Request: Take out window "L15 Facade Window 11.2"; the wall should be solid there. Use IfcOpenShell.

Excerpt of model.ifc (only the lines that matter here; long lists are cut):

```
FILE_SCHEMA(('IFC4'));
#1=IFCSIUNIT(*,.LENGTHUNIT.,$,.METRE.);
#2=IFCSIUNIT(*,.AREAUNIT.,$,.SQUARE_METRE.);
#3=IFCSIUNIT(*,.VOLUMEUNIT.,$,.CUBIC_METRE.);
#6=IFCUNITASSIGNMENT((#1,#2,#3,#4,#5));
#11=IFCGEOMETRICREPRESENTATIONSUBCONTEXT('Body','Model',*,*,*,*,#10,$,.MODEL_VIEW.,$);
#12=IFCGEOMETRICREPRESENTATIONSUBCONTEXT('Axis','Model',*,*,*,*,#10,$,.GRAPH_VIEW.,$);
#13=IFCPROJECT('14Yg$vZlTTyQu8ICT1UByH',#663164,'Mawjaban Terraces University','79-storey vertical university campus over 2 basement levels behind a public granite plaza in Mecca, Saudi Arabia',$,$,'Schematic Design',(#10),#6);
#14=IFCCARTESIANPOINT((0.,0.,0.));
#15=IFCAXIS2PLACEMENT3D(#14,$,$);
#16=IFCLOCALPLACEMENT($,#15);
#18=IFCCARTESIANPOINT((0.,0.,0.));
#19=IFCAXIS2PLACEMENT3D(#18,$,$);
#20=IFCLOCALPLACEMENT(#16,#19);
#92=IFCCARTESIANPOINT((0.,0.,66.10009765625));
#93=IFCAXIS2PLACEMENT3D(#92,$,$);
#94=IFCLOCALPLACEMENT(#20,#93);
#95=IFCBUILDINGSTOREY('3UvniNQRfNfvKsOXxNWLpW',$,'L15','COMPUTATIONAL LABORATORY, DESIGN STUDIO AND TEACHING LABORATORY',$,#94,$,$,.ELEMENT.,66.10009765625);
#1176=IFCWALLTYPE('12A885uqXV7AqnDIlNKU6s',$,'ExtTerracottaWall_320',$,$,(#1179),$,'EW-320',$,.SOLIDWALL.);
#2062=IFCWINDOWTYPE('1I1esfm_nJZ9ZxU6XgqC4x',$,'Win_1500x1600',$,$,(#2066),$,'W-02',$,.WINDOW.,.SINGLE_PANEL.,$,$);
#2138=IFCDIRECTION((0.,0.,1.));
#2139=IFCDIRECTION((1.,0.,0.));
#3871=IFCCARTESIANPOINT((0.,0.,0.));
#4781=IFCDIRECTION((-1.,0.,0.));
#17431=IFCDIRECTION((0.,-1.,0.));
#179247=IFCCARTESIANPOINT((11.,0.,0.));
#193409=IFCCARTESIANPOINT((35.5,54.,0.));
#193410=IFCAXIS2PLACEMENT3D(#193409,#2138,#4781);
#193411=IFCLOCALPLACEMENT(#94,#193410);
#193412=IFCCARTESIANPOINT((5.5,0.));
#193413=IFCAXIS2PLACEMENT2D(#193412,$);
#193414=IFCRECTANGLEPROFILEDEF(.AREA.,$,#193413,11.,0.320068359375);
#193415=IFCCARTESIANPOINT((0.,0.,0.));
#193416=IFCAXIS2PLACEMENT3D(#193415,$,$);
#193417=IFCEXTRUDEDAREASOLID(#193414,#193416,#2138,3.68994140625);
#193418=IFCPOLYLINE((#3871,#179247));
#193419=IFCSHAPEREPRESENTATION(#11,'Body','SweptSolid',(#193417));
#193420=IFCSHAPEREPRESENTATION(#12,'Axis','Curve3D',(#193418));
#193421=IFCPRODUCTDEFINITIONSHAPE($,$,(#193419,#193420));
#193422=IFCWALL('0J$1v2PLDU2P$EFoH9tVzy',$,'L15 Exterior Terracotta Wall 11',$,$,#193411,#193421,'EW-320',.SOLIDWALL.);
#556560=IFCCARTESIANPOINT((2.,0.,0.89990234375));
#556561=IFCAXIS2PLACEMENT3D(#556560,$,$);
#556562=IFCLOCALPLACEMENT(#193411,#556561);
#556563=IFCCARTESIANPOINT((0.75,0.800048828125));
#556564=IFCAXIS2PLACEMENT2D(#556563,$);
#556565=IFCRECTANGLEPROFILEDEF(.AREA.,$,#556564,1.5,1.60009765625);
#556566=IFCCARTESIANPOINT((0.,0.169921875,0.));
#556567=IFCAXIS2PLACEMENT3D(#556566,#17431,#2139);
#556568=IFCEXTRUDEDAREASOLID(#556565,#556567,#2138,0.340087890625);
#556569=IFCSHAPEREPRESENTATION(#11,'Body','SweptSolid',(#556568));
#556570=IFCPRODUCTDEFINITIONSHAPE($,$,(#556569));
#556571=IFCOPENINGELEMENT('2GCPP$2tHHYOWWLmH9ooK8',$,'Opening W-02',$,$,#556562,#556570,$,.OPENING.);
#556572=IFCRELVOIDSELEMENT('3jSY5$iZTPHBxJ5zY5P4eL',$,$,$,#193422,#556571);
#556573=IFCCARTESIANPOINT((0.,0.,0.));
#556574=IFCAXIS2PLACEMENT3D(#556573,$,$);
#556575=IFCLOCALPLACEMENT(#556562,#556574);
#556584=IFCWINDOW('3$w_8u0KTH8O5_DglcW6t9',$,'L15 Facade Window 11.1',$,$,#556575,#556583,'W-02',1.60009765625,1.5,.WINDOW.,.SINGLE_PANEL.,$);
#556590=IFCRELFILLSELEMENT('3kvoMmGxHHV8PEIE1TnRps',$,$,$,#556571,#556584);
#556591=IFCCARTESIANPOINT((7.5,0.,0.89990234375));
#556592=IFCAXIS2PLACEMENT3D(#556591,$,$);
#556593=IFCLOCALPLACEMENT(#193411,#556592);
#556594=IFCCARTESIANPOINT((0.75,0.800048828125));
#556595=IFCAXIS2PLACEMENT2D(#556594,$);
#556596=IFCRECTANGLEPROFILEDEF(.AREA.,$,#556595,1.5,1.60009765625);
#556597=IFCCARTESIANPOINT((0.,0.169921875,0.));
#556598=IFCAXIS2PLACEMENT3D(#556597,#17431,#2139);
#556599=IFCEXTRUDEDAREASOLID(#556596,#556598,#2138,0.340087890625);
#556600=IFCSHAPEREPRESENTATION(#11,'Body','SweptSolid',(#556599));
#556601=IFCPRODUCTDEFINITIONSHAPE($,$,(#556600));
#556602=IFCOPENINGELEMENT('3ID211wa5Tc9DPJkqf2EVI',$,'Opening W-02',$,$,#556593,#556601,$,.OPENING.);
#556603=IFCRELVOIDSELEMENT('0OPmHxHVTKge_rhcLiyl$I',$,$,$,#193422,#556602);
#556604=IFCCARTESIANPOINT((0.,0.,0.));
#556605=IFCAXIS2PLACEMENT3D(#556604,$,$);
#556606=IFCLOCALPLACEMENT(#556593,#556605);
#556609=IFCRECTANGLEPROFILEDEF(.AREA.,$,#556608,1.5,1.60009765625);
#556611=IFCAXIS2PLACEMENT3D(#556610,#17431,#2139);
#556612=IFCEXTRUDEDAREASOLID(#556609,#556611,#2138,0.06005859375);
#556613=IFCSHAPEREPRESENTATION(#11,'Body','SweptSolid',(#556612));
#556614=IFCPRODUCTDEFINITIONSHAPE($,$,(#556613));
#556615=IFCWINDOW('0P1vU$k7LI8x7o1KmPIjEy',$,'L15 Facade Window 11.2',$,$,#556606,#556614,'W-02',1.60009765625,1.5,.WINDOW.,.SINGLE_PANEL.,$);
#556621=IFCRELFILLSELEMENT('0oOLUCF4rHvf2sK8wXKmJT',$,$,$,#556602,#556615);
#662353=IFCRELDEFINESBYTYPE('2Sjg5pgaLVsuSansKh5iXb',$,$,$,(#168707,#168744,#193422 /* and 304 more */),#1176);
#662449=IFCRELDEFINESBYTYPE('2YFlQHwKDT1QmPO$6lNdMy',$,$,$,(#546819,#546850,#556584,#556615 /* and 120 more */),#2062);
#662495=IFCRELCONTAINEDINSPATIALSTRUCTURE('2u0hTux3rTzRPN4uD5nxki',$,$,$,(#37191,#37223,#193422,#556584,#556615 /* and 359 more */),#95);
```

```python
import ifcopenshell
import ifcopenshell.api.feature
import ifcopenshell.api.root
import ifcopenshell.geom
import ifcopenshell.util.shape

model = ifcopenshell.open("model.ifc")
settings = ifcopenshell.geom.settings()


def volume(element):
    """Net volume in cubic metres, openings subtracted."""
    shape = ifcopenshell.geom.create_shape(settings, element)
    return ifcopenshell.util.shape.get_volume(shape.geometry)


window = model.by_guid("0P1vU$k7LI8x7o1KmPIjEy")
opening = window.FillsVoids[0].RelatingOpeningElement
wall = opening.VoidsElements[0].RelatingBuildingElement
before = volume(wall)

ifcopenshell.api.root.remove_product(model, product=window)
ifcopenshell.api.feature.remove_feature(model, feature=opening)

after = volume(wall)

print(f"wall volume {before:.3f} -> {after:.3f} m3")

model.write("model_edited.ifc")
```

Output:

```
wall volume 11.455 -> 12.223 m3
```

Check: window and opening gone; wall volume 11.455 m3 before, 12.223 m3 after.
